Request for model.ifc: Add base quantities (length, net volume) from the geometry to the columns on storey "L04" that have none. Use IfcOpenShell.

First a look at what the model holds.

```python
import ifcopenshell
import ifcopenshell.util.element
import ifcopenshell.util.unit

model = ifcopenshell.open("model.ifc")
print(model.schema)
for unit_type in ("LENGTHUNIT", "AREAUNIT", "VOLUMEUNIT"):
    print(unit_type, ifcopenshell.util.unit.calculate_unit_scale(model, unit_type))
storey = next(s for s in model.by_type("IfcBuildingStorey") if s.Name == "L04")
columns = [e for e in ifcopenshell.util.element.get_decomposition(storey) if e.is_a("IfcColumn")]
for e in sorted(columns, key=lambda e: e.id()):
    print(e.id(), e.is_a(), e.Name, list(ifcopenshell.util.element.get_psets(e, qtos_only=True)), sep=" | ")
```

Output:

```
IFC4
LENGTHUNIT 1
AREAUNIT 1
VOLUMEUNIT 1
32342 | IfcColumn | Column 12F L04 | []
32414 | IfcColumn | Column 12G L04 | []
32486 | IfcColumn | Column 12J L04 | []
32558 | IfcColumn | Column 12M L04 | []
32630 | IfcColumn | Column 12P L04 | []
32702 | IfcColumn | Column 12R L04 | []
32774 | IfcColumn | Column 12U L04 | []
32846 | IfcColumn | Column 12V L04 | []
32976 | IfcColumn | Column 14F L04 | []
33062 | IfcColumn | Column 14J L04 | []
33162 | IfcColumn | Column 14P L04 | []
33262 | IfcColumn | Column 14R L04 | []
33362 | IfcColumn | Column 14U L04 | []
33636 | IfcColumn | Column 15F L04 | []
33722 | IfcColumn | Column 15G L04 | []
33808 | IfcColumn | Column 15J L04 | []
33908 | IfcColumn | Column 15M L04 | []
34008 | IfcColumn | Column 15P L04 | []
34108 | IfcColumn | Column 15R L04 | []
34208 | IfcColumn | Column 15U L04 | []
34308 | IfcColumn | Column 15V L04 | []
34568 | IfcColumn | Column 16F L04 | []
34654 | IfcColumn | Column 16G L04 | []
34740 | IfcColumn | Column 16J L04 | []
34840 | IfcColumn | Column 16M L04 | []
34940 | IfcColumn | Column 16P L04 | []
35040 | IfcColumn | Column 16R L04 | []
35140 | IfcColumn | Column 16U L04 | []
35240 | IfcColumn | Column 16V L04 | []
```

```python
import ifcopenshell
import ifcopenshell.api.pset
import ifcopenshell.geom
import ifcopenshell.util.element
import ifcopenshell.util.shape
import ifcopenshell.util.unit

model = ifcopenshell.open("model.ifc")
unit_scale = ifcopenshell.util.unit.calculate_unit_scale(model)
volume_scale = ifcopenshell.util.unit.calculate_unit_scale(model, "VOLUMEUNIT")
settings = ifcopenshell.geom.settings()

storey = next(s for s in model.by_type("IfcBuildingStorey") if s.Name == "L04")
columns = [e for e in ifcopenshell.util.element.get_decomposition(storey) if e.is_a("IfcColumn")]

for e in sorted(columns, key=lambda e: e.id()):
    if ifcopenshell.util.element.get_psets(e, qtos_only=True, should_inherit=False):
        continue
    # Geometry comes back in metres, in the element's own axes.
    shape = ifcopenshell.geom.create_shape(settings, e)
    values = {
        "Length": ifcopenshell.util.shape.get_z(shape.geometry) / unit_scale,
        "NetVolume": ifcopenshell.util.shape.get_volume(shape.geometry) / volume_scale,
    }
    qto = ifcopenshell.api.pset.add_qto(model, product=e, name="Qto_ColumnBaseQuantities")
    ifcopenshell.api.pset.edit_qto(model, qto=qto, properties=values)
    print(e.id(), {k: round(v, 3) for k, v in values.items()})

model.write("model_v2.ifc")
```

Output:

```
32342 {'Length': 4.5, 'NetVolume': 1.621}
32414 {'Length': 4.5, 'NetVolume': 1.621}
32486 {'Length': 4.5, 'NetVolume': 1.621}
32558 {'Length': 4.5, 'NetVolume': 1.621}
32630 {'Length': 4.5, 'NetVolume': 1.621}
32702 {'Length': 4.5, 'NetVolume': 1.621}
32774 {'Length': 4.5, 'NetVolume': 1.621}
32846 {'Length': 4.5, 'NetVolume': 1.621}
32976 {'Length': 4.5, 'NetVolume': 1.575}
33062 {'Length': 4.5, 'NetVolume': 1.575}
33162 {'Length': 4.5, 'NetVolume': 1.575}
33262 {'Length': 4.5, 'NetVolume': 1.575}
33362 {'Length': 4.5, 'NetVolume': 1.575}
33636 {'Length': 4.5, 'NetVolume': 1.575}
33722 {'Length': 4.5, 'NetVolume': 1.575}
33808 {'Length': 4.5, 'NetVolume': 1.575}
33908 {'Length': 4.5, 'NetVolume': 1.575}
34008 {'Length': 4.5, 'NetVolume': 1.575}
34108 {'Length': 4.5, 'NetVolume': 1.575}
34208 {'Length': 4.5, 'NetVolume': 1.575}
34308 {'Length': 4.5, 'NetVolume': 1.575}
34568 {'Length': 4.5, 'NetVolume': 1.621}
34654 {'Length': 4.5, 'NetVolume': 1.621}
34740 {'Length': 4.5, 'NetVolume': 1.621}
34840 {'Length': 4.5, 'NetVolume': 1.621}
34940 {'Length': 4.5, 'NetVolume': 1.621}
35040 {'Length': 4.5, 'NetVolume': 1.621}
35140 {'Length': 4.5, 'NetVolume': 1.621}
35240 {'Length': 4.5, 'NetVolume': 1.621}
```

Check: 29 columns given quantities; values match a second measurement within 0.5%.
